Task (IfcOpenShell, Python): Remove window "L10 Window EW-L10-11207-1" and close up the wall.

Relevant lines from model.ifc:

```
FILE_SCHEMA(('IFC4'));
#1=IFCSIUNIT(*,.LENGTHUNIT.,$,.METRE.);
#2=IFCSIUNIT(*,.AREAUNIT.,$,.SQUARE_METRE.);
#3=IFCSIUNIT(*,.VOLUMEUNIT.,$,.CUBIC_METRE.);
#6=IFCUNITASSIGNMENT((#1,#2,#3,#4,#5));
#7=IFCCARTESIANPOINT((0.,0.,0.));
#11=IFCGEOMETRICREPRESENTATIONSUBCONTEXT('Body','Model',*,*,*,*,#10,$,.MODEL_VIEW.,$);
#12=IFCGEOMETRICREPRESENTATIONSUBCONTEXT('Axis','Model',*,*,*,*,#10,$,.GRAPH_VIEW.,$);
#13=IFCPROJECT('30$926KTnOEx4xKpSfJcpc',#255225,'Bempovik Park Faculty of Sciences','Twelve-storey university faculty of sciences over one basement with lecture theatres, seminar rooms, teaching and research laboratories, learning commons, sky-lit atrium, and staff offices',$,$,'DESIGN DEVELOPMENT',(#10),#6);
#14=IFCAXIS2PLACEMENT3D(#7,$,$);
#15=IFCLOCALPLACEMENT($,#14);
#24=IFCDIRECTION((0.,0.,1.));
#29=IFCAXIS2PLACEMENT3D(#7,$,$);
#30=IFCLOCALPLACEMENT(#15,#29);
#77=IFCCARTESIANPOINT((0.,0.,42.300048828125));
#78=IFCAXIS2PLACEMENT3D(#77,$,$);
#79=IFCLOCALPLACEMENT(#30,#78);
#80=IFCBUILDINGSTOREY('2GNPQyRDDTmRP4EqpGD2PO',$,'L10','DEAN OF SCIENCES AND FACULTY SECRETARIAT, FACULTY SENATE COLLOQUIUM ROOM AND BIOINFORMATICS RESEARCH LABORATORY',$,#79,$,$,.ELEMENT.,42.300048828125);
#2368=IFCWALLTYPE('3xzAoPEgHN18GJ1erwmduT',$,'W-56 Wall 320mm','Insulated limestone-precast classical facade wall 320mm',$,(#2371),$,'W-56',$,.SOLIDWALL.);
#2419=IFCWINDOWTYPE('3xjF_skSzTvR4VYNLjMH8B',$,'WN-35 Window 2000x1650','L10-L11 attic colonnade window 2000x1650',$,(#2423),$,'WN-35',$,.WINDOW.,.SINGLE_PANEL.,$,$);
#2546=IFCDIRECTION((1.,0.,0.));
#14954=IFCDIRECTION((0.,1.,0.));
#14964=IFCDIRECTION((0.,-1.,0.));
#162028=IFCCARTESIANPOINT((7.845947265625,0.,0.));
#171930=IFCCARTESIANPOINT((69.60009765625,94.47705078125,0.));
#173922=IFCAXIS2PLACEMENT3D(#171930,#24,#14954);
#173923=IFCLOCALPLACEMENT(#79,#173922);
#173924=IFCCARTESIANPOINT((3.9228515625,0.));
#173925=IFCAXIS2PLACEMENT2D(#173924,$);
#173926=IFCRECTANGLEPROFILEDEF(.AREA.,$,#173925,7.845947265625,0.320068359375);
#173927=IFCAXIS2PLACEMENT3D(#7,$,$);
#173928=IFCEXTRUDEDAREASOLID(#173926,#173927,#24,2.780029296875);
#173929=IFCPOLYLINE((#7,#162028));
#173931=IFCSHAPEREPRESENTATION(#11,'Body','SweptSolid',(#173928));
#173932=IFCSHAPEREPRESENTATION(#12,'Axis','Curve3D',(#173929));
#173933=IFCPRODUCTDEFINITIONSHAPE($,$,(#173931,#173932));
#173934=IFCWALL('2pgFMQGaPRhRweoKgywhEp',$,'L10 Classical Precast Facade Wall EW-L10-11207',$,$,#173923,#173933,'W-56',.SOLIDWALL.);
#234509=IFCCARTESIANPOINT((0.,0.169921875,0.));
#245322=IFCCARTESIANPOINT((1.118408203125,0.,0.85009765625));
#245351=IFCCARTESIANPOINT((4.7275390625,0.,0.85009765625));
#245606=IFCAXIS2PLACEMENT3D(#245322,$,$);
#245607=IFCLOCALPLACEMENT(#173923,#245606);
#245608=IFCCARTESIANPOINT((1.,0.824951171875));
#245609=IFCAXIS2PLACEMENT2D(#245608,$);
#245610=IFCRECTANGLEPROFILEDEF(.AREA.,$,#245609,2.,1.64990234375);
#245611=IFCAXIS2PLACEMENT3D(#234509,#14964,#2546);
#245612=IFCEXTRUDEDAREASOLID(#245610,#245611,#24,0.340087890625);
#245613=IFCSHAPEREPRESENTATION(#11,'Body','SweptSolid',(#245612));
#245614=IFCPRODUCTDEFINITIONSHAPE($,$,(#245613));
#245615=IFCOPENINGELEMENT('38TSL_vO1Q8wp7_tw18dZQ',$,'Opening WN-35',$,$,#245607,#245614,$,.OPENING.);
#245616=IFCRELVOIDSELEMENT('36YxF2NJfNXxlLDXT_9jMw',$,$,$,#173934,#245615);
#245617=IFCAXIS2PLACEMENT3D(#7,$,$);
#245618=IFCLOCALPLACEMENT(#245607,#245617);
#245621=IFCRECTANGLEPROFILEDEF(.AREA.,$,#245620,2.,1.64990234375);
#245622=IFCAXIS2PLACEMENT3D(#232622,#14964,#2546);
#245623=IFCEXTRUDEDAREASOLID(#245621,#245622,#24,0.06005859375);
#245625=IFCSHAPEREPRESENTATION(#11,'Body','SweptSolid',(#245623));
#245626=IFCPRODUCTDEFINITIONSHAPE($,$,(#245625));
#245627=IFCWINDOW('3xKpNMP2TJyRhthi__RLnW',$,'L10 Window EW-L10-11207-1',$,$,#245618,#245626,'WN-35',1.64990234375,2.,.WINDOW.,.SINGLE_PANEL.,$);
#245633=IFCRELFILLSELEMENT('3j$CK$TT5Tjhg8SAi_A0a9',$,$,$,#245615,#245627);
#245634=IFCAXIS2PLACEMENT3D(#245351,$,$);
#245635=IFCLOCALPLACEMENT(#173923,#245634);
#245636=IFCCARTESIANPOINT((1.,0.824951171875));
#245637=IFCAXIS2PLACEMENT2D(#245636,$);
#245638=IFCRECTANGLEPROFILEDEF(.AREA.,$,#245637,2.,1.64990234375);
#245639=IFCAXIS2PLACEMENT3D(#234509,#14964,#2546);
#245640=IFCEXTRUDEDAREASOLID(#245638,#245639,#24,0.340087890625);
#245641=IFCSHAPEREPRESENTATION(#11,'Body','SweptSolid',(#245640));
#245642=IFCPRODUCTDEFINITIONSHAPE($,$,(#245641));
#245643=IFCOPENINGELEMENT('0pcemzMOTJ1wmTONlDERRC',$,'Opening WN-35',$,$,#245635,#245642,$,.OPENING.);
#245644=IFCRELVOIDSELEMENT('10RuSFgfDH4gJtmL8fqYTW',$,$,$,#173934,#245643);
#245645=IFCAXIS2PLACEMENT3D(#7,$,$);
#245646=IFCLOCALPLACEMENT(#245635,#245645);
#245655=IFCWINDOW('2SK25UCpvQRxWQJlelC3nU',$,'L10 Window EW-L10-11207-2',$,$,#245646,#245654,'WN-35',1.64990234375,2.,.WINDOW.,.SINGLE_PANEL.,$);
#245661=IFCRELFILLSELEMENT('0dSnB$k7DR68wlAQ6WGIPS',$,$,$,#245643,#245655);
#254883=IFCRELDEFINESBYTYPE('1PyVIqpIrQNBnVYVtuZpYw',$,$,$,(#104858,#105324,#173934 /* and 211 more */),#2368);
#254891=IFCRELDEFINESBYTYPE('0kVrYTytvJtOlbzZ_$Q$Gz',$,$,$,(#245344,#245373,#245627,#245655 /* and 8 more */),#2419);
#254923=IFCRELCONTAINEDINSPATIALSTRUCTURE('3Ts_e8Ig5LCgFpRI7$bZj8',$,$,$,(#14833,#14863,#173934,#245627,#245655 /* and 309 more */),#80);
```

```python
import ifcopenshell
import ifcopenshell.api.feature
import ifcopenshell.api.root
import ifcopenshell.geom
import ifcopenshell.util.shape

model = ifcopenshell.open("model.ifc")
settings = ifcopenshell.geom.settings()


def volume(element):
    """Net volume in cubic metres, openings subtracted."""
    shape = ifcopenshell.geom.create_shape(settings, element)
    return ifcopenshell.util.shape.get_volume(shape.geometry)


window = model.by_id(245627)
opening = window.FillsVoids[0].RelatingOpeningElement
wall = opening.VoidsElements[0].RelatingBuildingElement
before = volume(wall)

ifcopenshell.api.root.remove_product(model, product=window)
ifcopenshell.api.feature.remove_feature(model, feature=opening)

after = volume(wall)

print(f"wall volume {before:.3f} -> {after:.3f} m3")

model.write("model_rev.ifc")
```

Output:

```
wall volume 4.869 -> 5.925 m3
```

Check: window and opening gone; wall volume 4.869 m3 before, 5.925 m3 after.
